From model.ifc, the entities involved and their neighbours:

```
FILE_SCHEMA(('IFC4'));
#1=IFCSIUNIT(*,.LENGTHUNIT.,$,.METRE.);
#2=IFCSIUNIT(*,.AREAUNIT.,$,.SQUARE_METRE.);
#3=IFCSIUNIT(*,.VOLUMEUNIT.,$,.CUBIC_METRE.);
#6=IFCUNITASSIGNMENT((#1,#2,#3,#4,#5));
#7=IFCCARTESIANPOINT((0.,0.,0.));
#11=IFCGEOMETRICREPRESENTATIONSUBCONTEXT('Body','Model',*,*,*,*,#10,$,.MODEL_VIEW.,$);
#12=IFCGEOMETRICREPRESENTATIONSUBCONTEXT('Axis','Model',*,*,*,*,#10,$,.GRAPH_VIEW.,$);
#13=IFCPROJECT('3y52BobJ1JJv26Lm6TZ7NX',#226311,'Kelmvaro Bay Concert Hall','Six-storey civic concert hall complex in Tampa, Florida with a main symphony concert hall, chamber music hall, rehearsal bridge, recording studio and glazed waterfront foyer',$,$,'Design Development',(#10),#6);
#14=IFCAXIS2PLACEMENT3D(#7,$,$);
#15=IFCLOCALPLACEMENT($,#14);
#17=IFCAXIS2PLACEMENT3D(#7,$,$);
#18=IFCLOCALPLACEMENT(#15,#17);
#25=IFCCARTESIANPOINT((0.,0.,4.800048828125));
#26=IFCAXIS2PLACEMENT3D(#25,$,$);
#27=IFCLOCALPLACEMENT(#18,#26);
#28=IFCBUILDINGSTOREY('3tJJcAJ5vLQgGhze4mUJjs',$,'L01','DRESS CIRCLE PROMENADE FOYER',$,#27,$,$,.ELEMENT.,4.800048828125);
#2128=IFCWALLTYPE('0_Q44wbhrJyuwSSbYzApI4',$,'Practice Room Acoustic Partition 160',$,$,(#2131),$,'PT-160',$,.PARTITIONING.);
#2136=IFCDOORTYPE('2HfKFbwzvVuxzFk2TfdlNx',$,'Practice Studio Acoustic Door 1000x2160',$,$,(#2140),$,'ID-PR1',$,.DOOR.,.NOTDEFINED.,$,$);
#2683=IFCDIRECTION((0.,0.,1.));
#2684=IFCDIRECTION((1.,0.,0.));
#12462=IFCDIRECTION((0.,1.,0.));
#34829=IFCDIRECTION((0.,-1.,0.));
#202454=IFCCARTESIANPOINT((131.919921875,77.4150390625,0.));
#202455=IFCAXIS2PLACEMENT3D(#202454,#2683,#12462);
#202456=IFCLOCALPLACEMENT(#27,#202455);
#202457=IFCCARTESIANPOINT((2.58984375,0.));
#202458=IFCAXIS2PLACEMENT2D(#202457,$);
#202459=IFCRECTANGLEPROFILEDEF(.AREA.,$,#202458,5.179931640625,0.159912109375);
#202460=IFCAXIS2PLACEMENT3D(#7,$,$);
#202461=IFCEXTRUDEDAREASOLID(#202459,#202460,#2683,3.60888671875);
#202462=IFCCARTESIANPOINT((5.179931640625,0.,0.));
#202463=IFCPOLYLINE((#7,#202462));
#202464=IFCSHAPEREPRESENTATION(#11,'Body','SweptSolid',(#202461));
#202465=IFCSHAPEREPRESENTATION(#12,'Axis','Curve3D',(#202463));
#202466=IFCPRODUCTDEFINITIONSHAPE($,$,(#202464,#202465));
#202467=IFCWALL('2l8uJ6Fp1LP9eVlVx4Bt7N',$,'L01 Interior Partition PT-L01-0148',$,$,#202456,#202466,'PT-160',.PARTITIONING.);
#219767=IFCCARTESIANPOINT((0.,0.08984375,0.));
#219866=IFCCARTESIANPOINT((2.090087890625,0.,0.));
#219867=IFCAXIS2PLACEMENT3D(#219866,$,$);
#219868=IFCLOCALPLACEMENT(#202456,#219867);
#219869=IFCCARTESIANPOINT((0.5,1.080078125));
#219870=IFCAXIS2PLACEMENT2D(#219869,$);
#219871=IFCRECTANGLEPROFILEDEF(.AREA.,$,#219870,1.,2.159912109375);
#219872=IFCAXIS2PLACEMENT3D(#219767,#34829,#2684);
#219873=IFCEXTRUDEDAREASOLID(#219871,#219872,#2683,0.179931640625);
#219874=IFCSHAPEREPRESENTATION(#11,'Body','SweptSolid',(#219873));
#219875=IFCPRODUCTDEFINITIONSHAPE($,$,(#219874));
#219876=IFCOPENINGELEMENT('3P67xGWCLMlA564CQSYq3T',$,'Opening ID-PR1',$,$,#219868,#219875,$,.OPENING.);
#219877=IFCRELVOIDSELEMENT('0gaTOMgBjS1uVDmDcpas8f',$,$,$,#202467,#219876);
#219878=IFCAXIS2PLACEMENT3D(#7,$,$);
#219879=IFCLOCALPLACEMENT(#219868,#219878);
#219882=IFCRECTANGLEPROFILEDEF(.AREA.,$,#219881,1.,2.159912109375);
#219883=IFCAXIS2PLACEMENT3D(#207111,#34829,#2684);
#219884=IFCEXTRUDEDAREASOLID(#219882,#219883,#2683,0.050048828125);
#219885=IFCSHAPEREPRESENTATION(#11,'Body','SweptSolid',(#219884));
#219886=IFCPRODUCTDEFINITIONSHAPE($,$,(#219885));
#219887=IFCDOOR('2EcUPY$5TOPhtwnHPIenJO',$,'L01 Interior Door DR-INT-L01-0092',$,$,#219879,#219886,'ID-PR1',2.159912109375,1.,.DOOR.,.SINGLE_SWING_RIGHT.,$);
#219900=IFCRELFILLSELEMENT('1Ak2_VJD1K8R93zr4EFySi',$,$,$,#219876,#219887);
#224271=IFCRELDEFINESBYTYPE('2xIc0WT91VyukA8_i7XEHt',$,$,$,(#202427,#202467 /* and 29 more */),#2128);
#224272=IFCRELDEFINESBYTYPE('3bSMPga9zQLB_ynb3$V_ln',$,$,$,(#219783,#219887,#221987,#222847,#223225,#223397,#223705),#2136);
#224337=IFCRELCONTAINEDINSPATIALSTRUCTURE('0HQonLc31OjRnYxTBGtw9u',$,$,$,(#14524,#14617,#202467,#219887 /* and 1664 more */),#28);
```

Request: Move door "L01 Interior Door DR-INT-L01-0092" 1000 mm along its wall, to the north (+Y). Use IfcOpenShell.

```python
import ifcopenshell
import ifcopenshell.api.geometry
import ifcopenshell.util.placement
import ifcopenshell.util.unit

model = ifcopenshell.open("model.ifc")
unit_scale = ifcopenshell.util.unit.calculate_unit_scale(model)

door = model.by_guid("2EcUPY$5TOPhtwnHPIenJO")
opening = door.FillsVoids[0].RelatingOpeningElement
wall = opening.VoidsElements[0].RelatingBuildingElement

wall_matrix = ifcopenshell.util.placement.get_local_placement(wall.ObjectPlacement)
shift = wall_matrix[:3, 0] * 1 / unit_scale
before = ifcopenshell.util.placement.get_local_placement(door.ObjectPlacement)[:3, 3].copy()

# The door is placed relative to its opening, so it follows when the opening moves.
matrix = ifcopenshell.util.placement.get_local_placement(opening.ObjectPlacement)
matrix[:3, 3] += shift
ifcopenshell.api.geometry.edit_object_placement(
    model, product=opening, matrix=matrix, is_si=False, should_transform_children=True
)

after = ifcopenshell.util.placement.get_local_placement(door.ObjectPlacement)[:3, 3]
print("door moved by", (after - before).round(3) + 0.0)

model.write("model_v2.ifc")
```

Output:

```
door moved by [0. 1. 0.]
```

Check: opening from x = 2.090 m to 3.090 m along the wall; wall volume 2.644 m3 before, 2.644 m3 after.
